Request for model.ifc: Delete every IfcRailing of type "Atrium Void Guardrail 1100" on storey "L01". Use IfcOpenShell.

First a look at what the model holds.

```python
import ifcopenshell
import ifcopenshell.util.element

model = ifcopenshell.open("model.ifc")
print(model.schema)
storey = next(s for s in model.by_type("IfcBuildingStorey") if s.Name == "L01")
railings = [e for e in ifcopenshell.util.element.get_decomposition(storey) if e.is_a("IfcRailing")]
seen = {}
for e in railings:
    element_type = ifcopenshell.util.element.get_type(e)
    name = element_type.Name if element_type not in (None, e) else None
    seen[name] = seen.get(name, 0) + 1
for name, count in sorted(seen.items(), key=str):
    print(count, "x", name)
```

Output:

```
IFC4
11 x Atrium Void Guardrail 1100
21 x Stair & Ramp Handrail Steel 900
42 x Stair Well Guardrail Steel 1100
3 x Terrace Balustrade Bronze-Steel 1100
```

```python
import ifcopenshell
import ifcopenshell.api.root
import ifcopenshell.util.element

model = ifcopenshell.open("model.ifc")

storey = next(s for s in model.by_type("IfcBuildingStorey") if s.Name == "L01")
railings = [e for e in ifcopenshell.util.element.get_decomposition(storey) if e.is_a("IfcRailing")]
targets = [e for e in railings if (t := ifcopenshell.util.element.get_type(e)) not in (None, e) and t.Name == "Atrium Void Guardrail 1100"]

for e in targets:
    ifcopenshell.api.root.remove_product(model, product=e)
print(len(targets), "removed")

model.write("model_v2.ifc")
```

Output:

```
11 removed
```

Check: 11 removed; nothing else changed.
